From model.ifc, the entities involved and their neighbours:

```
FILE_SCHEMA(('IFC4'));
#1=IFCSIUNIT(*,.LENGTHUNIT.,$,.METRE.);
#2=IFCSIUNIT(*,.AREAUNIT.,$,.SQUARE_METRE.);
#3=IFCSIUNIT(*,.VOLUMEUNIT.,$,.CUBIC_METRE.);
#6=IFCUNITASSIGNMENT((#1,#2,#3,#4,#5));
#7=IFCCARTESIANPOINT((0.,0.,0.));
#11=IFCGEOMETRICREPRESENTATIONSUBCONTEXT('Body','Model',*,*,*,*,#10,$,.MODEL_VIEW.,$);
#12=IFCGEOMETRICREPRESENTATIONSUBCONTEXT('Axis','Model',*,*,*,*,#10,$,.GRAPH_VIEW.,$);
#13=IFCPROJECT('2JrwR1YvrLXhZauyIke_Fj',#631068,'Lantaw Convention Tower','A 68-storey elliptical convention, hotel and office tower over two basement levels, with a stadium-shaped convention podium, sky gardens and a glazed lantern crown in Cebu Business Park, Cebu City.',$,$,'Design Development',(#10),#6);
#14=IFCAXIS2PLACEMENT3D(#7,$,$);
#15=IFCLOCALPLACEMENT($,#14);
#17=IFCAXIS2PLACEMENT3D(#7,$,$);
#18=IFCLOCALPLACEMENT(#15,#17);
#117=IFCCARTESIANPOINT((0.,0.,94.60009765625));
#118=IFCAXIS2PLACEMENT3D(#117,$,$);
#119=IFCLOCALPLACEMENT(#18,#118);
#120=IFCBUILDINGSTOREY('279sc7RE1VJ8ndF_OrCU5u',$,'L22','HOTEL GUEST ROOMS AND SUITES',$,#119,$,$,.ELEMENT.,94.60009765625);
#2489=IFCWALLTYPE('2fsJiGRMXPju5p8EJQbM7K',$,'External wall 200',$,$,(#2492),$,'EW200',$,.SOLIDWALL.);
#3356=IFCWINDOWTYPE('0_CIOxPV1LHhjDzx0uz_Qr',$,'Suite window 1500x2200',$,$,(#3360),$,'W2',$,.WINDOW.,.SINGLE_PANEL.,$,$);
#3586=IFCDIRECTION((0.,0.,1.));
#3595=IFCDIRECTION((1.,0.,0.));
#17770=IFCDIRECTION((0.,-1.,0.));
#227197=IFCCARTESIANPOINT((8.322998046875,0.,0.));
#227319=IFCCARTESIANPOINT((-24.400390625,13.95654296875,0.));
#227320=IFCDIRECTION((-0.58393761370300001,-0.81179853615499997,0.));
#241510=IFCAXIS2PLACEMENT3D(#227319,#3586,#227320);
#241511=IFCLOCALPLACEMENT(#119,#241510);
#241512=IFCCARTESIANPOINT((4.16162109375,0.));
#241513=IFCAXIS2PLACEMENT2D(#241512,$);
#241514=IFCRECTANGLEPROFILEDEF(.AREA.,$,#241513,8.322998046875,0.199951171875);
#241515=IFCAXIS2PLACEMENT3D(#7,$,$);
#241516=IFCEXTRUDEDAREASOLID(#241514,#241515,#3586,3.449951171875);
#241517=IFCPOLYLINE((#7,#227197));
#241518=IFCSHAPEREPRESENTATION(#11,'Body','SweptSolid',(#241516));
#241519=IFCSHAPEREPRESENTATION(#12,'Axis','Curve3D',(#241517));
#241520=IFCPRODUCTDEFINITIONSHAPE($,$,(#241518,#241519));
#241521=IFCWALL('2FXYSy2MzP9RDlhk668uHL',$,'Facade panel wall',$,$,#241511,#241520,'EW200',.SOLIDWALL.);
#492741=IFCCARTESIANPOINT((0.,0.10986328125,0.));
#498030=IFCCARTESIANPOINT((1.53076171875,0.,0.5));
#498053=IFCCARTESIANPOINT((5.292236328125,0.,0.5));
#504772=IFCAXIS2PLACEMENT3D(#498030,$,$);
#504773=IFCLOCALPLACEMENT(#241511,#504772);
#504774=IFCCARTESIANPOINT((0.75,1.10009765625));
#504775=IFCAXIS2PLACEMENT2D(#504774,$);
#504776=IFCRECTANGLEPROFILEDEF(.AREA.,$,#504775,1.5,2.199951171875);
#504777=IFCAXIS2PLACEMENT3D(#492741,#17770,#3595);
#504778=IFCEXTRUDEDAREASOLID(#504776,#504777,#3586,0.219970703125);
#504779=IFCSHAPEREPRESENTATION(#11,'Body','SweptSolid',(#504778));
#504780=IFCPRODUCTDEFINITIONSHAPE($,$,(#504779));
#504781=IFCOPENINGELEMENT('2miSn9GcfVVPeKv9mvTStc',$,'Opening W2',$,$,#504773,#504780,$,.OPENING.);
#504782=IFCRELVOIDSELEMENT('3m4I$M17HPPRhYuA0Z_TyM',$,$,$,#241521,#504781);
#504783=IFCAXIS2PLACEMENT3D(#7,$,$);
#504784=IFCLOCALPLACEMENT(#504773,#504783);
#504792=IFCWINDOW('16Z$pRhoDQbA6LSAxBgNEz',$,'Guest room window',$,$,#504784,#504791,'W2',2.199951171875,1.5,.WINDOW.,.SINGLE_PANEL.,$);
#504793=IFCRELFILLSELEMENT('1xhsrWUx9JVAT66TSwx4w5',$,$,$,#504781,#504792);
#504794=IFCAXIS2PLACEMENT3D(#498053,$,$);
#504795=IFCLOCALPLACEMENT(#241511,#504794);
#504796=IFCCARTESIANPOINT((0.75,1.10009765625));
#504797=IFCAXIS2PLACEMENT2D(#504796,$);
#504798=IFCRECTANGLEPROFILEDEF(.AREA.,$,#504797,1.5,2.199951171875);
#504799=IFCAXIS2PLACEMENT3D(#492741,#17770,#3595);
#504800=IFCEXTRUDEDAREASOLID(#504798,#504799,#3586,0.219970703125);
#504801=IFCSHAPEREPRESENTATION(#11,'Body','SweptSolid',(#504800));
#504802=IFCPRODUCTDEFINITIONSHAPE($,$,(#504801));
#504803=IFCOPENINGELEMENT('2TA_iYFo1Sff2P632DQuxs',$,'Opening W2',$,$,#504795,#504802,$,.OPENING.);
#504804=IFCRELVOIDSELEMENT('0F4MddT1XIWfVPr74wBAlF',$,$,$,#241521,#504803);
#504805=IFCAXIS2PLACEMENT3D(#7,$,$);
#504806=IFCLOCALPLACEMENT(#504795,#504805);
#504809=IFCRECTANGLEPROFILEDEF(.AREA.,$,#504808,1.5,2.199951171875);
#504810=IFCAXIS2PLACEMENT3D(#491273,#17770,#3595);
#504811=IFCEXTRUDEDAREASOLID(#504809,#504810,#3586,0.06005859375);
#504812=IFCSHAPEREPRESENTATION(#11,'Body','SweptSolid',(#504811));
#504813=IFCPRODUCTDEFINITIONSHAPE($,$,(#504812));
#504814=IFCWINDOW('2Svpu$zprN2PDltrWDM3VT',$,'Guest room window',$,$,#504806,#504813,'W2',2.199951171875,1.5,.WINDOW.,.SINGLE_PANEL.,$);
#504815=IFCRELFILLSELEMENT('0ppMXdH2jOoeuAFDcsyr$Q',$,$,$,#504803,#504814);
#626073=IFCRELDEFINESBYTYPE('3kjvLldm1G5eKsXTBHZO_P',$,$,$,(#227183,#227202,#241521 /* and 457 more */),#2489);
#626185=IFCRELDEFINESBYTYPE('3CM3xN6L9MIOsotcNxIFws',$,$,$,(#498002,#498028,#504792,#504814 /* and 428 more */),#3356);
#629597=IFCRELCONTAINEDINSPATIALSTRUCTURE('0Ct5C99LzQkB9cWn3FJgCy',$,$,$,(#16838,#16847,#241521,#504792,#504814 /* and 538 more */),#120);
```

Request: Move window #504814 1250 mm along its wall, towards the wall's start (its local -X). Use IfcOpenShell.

```python
import ifcopenshell
import ifcopenshell.api.geometry
import ifcopenshell.util.placement
import ifcopenshell.util.unit

model = ifcopenshell.open("model.ifc")
unit_scale = ifcopenshell.util.unit.calculate_unit_scale(model)

window = model.by_guid("2Svpu$zprN2PDltrWDM3VT")
opening = window.FillsVoids[0].RelatingOpeningElement
wall = opening.VoidsElements[0].RelatingBuildingElement

wall_matrix = ifcopenshell.util.placement.get_local_placement(wall.ObjectPlacement)
shift = wall_matrix[:3, 0] * -1.25 / unit_scale
before = ifcopenshell.util.placement.get_local_placement(window.ObjectPlacement)[:3, 3].copy()

# The window is placed relative to its opening, so it follows when the opening moves.
matrix = ifcopenshell.util.placement.get_local_placement(opening.ObjectPlacement)
matrix[:3, 3] += shift
ifcopenshell.api.geometry.edit_object_placement(
    model, product=opening, matrix=matrix, is_si=False, should_transform_children=True
)

after = ifcopenshell.util.placement.get_local_placement(window.ObjectPlacement)[:3, 3]
print("window moved by", (after - before).round(3) + 0.0)

model.write("model_v2.ifc")
```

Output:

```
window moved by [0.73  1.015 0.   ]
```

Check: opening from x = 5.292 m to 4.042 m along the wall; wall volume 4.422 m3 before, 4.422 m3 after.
